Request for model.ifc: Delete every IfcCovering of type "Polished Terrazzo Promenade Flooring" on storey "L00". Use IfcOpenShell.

First a look at what the model holds.

```python
import ifcopenshell
import ifcopenshell.util.element

model = ifcopenshell.open("model.ifc")
print(model.schema)
storey = next(s for s in model.by_type("IfcBuildingStorey") if s.Name == "L00")
coverings = [e for e in ifcopenshell.util.element.get_decomposition(storey) if e.is_a("IfcCovering")]
seen = {}
for e in coverings:
    element_type = ifcopenshell.util.element.get_type(e)
    name = element_type.Name if element_type not in (None, e) else None
    seen[name] = seen.get(name, 0) + 1
for name, count in sorted(seen.items(), key=str):
    print(count, "x", name)
```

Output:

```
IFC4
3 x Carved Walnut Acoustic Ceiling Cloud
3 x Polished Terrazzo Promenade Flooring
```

```python
import ifcopenshell
import ifcopenshell.api.root
import ifcopenshell.util.element

model = ifcopenshell.open("model.ifc")

storey = next(s for s in model.by_type("IfcBuildingStorey") if s.Name == "L00")
coverings = [e for e in ifcopenshell.util.element.get_decomposition(storey) if e.is_a("IfcCovering")]
targets = [e for e in coverings if (t := ifcopenshell.util.element.get_type(e)) not in (None, e) and t.Name == "Polished Terrazzo Promenade Flooring"]

for e in targets:
    ifcopenshell.api.root.remove_product(model, product=e)
print(len(targets), "removed")

model.write("model_updated.ifc")
```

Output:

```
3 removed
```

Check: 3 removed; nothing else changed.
